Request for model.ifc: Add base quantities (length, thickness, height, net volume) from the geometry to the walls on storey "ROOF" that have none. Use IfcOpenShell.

First a look at what the model holds.

```python
import ifcopenshell
import ifcopenshell.util.element
import ifcopenshell.util.unit

model = ifcopenshell.open("model.ifc")
print(model.schema)
for unit_type in ("LENGTHUNIT", "AREAUNIT", "VOLUMEUNIT"):
    print(unit_type, ifcopenshell.util.unit.calculate_unit_scale(model, unit_type))
storey = next(s for s in model.by_type("IfcBuildingStorey") if s.Name == "ROOF")
walls = [e for e in ifcopenshell.util.element.get_decomposition(storey) if e.is_a("IfcWall")]
for e in sorted(walls, key=lambda e: e.id()):
    print(e.id(), e.is_a(), e.Name, list(ifcopenshell.util.element.get_psets(e, qtos_only=True)), sep=" | ")
```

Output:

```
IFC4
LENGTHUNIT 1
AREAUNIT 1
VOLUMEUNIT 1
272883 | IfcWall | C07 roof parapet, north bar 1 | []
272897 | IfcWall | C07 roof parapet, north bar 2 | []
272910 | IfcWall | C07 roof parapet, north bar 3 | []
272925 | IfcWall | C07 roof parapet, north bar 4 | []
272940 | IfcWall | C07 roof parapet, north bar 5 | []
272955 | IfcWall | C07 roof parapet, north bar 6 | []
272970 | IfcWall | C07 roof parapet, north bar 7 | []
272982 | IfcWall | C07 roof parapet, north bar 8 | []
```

```python
import ifcopenshell
import ifcopenshell.api.pset
import ifcopenshell.geom
import ifcopenshell.util.element
import ifcopenshell.util.shape
import ifcopenshell.util.unit

model = ifcopenshell.open("model.ifc")
unit_scale = ifcopenshell.util.unit.calculate_unit_scale(model)
volume_scale = ifcopenshell.util.unit.calculate_unit_scale(model, "VOLUMEUNIT")
settings = ifcopenshell.geom.settings()

storey = next(s for s in model.by_type("IfcBuildingStorey") if s.Name == "ROOF")
walls = [e for e in ifcopenshell.util.element.get_decomposition(storey) if e.is_a("IfcWall")]

for e in sorted(walls, key=lambda e: e.id()):
    if ifcopenshell.util.element.get_psets(e, qtos_only=True, should_inherit=False):
        continue
    # Geometry comes back in metres, in the element's own axes.
    shape = ifcopenshell.geom.create_shape(settings, e)
    values = {
        "Length": ifcopenshell.util.shape.get_x(shape.geometry) / unit_scale,
        "Width": ifcopenshell.util.shape.get_y(shape.geometry) / unit_scale,
        "Height": ifcopenshell.util.shape.get_z(shape.geometry) / unit_scale,
        "NetVolume": ifcopenshell.util.shape.get_volume(shape.geometry) / volume_scale,
    }
    qto = ifcopenshell.api.pset.add_qto(model, product=e, name="Qto_WallBaseQuantities")
    ifcopenshell.api.pset.edit_qto(model, qto=qto, properties=values)
    print(e.id(), {k: round(v, 3) for k, v in values.items()})

model.write("model-out.ifc")
```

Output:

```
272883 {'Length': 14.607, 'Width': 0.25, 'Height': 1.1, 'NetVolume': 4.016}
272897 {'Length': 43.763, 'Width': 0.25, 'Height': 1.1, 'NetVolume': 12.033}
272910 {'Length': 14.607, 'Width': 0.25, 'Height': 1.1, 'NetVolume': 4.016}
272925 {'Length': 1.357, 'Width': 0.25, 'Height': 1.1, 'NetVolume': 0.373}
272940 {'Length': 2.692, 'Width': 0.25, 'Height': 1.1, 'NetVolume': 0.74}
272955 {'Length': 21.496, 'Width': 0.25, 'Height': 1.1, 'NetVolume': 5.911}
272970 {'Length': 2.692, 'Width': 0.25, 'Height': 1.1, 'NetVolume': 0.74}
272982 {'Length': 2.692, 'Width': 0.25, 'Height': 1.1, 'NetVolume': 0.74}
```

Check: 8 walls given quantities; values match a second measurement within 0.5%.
